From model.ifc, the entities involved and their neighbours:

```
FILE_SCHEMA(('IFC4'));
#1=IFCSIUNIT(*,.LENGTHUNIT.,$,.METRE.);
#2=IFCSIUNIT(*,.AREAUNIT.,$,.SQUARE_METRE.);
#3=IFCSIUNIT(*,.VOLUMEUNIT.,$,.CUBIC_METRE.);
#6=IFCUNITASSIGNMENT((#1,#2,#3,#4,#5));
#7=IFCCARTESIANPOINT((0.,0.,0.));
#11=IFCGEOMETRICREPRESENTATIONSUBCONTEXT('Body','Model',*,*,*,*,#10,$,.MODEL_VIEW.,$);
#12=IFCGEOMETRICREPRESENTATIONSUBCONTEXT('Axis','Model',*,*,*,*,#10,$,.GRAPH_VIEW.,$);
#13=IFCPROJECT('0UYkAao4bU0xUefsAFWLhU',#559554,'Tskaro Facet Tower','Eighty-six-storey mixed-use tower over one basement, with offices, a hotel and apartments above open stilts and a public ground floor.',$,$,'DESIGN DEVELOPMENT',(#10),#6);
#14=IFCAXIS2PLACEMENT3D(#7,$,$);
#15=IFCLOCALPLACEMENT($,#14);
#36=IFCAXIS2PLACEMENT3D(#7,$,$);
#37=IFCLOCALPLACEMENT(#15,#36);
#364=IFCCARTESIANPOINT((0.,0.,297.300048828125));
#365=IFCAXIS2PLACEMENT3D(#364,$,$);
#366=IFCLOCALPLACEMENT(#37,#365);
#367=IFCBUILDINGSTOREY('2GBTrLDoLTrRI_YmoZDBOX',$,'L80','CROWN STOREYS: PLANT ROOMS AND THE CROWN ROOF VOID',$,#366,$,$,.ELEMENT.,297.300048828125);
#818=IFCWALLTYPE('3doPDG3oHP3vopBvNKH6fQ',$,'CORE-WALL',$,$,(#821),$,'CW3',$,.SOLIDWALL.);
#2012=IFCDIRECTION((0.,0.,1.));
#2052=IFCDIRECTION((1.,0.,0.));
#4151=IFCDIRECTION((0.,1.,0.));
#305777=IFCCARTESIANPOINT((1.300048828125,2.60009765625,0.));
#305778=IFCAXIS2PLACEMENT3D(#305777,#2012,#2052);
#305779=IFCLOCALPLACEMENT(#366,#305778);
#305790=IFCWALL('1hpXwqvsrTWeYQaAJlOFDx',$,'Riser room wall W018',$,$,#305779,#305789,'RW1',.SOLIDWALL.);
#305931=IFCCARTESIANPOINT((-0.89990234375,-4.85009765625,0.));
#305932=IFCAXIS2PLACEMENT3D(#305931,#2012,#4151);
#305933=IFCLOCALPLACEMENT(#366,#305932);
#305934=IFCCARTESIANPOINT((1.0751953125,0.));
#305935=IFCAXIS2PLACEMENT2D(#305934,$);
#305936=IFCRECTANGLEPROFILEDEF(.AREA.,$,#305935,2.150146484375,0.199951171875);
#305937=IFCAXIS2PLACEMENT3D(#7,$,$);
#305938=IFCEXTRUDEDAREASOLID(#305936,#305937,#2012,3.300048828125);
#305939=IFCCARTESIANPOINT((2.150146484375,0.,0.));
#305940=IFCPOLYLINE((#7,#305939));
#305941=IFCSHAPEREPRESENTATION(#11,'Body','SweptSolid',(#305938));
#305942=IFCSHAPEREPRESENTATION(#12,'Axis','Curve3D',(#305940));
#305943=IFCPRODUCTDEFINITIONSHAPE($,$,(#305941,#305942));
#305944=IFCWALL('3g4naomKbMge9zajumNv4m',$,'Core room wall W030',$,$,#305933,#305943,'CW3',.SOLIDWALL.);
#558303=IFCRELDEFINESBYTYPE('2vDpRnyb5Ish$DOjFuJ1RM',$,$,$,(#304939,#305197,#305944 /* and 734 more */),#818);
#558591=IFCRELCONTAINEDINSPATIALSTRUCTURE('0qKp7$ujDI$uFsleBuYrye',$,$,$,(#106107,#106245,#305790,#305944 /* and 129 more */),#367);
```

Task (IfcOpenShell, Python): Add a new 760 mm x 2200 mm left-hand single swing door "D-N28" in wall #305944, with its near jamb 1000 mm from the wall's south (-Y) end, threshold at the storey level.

```python
import numpy as np
import ifcopenshell
import ifcopenshell.api.feature
import ifcopenshell.api.geometry
import ifcopenshell.api.root
import ifcopenshell.api.spatial
import ifcopenshell.geom
import ifcopenshell.util.element
import ifcopenshell.util.placement
import ifcopenshell.util.representation
import ifcopenshell.util.shape
import ifcopenshell.util.unit

model = ifcopenshell.open("model.ifc")
unit_scale = ifcopenshell.util.unit.calculate_unit_scale(model)
settings = ifcopenshell.geom.settings()


def volume(element):
    """Net volume in cubic metres, openings subtracted."""
    shape = ifcopenshell.geom.create_shape(settings, element)
    return ifcopenshell.util.shape.get_volume(shape.geometry)


wall = model.by_guid("3g4naomKbMge9zajumNv4m")
storey = ifcopenshell.util.element.get_container(wall, ifc_class="IfcBuildingStorey")
context = ifcopenshell.util.representation.get_context(model, "Model", "Body", "MODEL_VIEW")
before = volume(wall)

width, height, from_end, sill = 0.76, 2.2, 1, 0.0  # metres

# The wall runs along its own X axis, and the end named is its -X end.
wall_shape = ifcopenshell.geom.create_shape(settings, wall)
x, y, z = ifcopenshell.util.shape.get_vertices(wall_shape.geometry).T
start = x.min() + from_end
face, thickness = float(y.min()), float(y.max() - y.min())
wall_matrix = ifcopenshell.util.placement.get_local_placement(wall.ObjectPlacement)
level = ifcopenshell.util.placement.get_local_placement(storey.ObjectPlacement)[2, 3]


def in_wall(x, y):
    """Placement at x, y metres in the wall's axes, at sill height."""
    matrix = wall_matrix.copy()
    matrix[:, 3] = wall_matrix @ np.array([x / unit_scale, y / unit_scale, 0.0, 1.0])
    matrix[2, 3] = level + sill / unit_scale
    return matrix


# Opening: a box that overshoots both wall faces by 50 mm.
opening = ifcopenshell.api.root.create_entity(model, ifc_class="IfcOpeningElement", predefined_type="OPENING")
box = ifcopenshell.api.geometry.add_wall_representation(
    model, context=context, length=width, height=height, thickness=thickness + 0.1
)
ifcopenshell.api.geometry.assign_representation(model, product=opening, representation=box)
ifcopenshell.api.geometry.edit_object_placement(model, product=opening, matrix=in_wall(start, face - 0.05), is_si=False)
ifcopenshell.api.feature.add_feature(model, feature=opening, element=wall)

door = ifcopenshell.api.root.create_entity(model, ifc_class="IfcDoor", name="D-N28", predefined_type="DOOR")
door.OverallWidth, door.OverallHeight = width / unit_scale, height / unit_scale
door.OperationType = "SINGLE_SWING_LEFT"
body = ifcopenshell.api.geometry.add_door_representation(
    model,
    context=context,
    overall_width=door.OverallWidth,
    overall_height=door.OverallHeight,
    operation_type="SINGLE_SWING_LEFT",
    lining_properties={"LiningDepth": thickness / unit_scale, "ThresholdDepth": thickness / unit_scale},
)
ifcopenshell.api.geometry.assign_representation(model, product=door, representation=body)
ifcopenshell.api.spatial.assign_container(model, products=[door], relating_structure=storey)
ifcopenshell.api.feature.add_filling(model, opening=opening, element=door)

# The lining spans the wall, so the door starts at the wall face.
ifcopenshell.api.geometry.edit_object_placement(model, product=door, matrix=in_wall(start, face), is_si=False)

after = volume(wall)

print(f"wall volume {before:.3f} -> {after:.3f} m3")

model.write("model_v2.ifc")
```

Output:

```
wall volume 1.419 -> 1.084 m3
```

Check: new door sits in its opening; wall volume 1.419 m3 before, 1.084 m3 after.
